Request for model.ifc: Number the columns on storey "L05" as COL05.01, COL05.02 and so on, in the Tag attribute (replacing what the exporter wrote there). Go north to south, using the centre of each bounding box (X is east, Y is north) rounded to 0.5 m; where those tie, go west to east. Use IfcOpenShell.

First a look at what the model holds.

```python
import ifcopenshell
import ifcopenshell.util.element
import ifcopenshell.util.placement

model = ifcopenshell.open("model.ifc")
print(model.schema)
storey = next(s for s in model.by_type("IfcBuildingStorey") if s.Name == "L05")
columns = [e for e in ifcopenshell.util.element.get_decomposition(storey) if e.is_a("IfcColumn")]
for e in sorted(columns, key=lambda e: e.id()):
    origin = ifcopenshell.util.placement.get_local_placement(e.ObjectPlacement)[:3, 3]
    print(e.id(), e.Tag, e.Name, origin.round(2) + 0.0, sep=" | ")
```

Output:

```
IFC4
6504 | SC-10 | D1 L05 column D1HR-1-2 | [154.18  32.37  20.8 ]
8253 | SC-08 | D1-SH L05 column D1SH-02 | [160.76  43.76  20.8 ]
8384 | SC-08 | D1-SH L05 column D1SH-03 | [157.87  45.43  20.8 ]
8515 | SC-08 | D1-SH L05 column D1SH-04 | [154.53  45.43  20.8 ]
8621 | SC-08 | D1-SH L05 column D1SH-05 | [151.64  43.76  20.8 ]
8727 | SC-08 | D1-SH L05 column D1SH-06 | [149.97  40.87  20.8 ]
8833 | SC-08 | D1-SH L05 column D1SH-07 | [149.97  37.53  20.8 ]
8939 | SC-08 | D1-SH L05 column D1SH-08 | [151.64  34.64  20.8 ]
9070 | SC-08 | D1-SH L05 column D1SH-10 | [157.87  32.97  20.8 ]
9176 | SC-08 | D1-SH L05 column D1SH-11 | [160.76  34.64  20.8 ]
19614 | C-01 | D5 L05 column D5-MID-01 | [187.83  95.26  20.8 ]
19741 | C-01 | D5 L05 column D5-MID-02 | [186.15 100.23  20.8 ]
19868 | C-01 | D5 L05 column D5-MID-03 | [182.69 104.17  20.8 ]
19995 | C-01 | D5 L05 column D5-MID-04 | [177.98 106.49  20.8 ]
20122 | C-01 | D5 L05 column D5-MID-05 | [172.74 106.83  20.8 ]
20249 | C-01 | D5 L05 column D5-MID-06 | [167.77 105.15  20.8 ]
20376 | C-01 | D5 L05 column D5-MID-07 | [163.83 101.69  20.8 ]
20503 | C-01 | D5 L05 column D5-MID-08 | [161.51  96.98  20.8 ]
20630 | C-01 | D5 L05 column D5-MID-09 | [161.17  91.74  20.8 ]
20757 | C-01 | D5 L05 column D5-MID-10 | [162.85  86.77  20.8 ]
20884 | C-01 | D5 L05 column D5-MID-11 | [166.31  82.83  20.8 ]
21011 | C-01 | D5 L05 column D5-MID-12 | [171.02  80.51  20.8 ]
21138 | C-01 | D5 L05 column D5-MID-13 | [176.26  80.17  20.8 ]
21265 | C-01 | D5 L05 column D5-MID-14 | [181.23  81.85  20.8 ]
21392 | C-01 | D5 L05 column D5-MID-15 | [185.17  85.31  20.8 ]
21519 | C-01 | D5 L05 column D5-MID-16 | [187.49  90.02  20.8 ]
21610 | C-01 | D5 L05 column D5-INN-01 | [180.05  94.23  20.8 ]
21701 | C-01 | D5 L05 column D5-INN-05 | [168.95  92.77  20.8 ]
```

```python
import ifcopenshell
import ifcopenshell.geom
import ifcopenshell.util.element
import ifcopenshell.util.shape

model = ifcopenshell.open("model.ifc")
settings = ifcopenshell.geom.settings()
settings.set("use-world-coords", True)


def centre(element):
    shape = ifcopenshell.geom.create_shape(settings, element)
    return ifcopenshell.util.shape.get_bbox_centroid(shape.geometry)


storey = next(s for s in model.by_type("IfcBuildingStorey") if s.Name == "L05")
columns = [e for e in ifcopenshell.util.element.get_decomposition(storey) if e.is_a("IfcColumn")]

# Insertion points can sit at a corner or the storey origin, so sort by the geometry (in metres).
centres = {e: centre(e) for e in columns}
columns.sort(key=lambda e: (-round(centres[e][1] / 0.5), centres[e][0]))

for i, e in enumerate(columns, start=1):
    number = f"COL05.{i:02d}"
    e.Tag = number
    print(e.id(), number)

model.write("model_updated.ifc")
```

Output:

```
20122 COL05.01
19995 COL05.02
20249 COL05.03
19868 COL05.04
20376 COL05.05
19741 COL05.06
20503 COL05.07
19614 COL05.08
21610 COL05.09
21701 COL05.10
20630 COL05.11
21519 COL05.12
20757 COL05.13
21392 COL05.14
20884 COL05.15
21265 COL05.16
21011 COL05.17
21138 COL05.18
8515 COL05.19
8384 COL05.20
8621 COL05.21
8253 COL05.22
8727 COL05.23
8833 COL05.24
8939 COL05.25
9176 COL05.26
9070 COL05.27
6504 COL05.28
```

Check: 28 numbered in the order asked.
